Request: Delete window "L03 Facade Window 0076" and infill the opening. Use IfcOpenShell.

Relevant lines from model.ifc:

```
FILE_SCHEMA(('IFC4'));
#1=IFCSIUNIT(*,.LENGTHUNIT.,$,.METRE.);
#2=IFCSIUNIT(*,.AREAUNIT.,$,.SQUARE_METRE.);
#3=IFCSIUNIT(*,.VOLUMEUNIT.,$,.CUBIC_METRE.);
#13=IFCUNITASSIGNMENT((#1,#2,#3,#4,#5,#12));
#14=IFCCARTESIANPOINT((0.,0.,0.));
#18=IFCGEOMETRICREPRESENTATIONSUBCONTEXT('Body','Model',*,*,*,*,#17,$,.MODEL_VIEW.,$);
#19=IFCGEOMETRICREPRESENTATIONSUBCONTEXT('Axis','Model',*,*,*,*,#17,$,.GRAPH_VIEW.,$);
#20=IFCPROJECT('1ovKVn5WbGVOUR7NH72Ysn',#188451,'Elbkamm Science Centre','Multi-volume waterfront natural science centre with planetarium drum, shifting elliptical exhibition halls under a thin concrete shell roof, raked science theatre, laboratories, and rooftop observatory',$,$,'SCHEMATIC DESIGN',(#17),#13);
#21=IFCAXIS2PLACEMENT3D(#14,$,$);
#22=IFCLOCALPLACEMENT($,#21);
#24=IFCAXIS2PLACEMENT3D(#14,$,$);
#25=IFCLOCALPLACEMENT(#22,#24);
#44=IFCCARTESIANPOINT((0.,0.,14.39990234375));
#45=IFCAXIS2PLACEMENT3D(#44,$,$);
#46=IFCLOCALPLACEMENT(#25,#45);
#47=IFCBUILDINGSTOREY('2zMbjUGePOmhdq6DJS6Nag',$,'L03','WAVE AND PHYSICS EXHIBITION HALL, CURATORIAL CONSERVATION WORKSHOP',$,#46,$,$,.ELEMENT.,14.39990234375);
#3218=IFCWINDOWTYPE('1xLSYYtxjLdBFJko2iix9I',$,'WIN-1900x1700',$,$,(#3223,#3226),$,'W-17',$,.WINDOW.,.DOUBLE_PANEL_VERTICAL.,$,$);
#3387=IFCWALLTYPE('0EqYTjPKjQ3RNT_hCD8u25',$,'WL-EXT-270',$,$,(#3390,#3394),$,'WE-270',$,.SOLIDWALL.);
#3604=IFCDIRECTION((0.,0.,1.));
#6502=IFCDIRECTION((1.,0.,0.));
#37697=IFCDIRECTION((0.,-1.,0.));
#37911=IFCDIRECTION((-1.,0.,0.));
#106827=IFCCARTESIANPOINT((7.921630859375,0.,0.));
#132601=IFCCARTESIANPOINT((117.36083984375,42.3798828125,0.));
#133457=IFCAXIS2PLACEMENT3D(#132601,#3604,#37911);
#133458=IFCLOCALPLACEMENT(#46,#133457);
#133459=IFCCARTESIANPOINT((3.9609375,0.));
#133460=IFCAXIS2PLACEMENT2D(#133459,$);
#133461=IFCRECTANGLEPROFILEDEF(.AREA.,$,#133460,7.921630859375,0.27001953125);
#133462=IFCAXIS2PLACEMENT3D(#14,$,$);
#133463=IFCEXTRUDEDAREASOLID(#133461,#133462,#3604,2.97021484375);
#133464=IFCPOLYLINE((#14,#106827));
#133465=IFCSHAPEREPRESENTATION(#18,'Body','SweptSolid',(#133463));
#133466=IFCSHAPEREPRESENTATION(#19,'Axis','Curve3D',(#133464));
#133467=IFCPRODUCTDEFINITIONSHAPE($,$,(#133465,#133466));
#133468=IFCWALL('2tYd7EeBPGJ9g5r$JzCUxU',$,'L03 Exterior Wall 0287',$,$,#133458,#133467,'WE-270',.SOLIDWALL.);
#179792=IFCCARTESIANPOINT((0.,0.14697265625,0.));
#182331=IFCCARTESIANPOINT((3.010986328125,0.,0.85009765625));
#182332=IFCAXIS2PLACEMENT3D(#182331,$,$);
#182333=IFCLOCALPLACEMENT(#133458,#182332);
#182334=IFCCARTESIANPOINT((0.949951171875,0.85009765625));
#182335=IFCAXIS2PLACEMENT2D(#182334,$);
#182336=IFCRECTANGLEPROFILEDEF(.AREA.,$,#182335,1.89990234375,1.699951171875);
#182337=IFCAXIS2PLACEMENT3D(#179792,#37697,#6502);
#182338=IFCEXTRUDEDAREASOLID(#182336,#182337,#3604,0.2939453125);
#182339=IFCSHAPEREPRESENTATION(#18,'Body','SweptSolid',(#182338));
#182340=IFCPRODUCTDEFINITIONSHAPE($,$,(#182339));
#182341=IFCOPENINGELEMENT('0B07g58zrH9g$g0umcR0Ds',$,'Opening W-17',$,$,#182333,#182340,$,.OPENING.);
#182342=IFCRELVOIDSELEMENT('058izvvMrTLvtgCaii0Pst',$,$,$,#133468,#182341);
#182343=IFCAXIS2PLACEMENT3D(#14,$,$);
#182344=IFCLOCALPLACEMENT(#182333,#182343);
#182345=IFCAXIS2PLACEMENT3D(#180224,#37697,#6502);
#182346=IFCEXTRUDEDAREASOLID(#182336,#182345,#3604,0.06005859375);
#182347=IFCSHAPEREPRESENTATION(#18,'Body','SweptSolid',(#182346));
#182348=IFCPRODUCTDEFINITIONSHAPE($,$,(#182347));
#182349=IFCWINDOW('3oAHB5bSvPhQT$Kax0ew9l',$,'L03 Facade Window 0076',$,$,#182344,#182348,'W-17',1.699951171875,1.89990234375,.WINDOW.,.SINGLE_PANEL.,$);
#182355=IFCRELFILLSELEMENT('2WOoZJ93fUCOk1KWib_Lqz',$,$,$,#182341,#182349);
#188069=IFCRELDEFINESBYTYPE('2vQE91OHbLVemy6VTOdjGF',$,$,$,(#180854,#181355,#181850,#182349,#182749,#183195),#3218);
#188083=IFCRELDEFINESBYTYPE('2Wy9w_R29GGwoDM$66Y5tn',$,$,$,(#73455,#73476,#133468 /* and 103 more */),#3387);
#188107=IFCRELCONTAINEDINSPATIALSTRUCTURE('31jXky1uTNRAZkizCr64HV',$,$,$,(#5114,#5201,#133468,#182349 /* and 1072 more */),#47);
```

```python
import ifcopenshell
import ifcopenshell.api.feature
import ifcopenshell.api.root
import ifcopenshell.geom
import ifcopenshell.util.shape

model = ifcopenshell.open("model.ifc")
settings = ifcopenshell.geom.settings()


def volume(element):
    """Net volume in cubic metres, openings subtracted."""
    shape = ifcopenshell.geom.create_shape(settings, element)
    return ifcopenshell.util.shape.get_volume(shape.geometry)


window = model.by_id(182349)
opening = window.FillsVoids[0].RelatingOpeningElement
wall = opening.VoidsElements[0].RelatingBuildingElement
before = volume(wall)

ifcopenshell.api.root.remove_product(model, product=window)
ifcopenshell.api.feature.remove_feature(model, feature=opening)

after = volume(wall)

print(f"wall volume {before:.3f} -> {after:.3f} m3")

model.write("model_v2.ifc")
```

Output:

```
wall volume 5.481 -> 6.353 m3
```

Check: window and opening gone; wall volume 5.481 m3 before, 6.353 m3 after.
